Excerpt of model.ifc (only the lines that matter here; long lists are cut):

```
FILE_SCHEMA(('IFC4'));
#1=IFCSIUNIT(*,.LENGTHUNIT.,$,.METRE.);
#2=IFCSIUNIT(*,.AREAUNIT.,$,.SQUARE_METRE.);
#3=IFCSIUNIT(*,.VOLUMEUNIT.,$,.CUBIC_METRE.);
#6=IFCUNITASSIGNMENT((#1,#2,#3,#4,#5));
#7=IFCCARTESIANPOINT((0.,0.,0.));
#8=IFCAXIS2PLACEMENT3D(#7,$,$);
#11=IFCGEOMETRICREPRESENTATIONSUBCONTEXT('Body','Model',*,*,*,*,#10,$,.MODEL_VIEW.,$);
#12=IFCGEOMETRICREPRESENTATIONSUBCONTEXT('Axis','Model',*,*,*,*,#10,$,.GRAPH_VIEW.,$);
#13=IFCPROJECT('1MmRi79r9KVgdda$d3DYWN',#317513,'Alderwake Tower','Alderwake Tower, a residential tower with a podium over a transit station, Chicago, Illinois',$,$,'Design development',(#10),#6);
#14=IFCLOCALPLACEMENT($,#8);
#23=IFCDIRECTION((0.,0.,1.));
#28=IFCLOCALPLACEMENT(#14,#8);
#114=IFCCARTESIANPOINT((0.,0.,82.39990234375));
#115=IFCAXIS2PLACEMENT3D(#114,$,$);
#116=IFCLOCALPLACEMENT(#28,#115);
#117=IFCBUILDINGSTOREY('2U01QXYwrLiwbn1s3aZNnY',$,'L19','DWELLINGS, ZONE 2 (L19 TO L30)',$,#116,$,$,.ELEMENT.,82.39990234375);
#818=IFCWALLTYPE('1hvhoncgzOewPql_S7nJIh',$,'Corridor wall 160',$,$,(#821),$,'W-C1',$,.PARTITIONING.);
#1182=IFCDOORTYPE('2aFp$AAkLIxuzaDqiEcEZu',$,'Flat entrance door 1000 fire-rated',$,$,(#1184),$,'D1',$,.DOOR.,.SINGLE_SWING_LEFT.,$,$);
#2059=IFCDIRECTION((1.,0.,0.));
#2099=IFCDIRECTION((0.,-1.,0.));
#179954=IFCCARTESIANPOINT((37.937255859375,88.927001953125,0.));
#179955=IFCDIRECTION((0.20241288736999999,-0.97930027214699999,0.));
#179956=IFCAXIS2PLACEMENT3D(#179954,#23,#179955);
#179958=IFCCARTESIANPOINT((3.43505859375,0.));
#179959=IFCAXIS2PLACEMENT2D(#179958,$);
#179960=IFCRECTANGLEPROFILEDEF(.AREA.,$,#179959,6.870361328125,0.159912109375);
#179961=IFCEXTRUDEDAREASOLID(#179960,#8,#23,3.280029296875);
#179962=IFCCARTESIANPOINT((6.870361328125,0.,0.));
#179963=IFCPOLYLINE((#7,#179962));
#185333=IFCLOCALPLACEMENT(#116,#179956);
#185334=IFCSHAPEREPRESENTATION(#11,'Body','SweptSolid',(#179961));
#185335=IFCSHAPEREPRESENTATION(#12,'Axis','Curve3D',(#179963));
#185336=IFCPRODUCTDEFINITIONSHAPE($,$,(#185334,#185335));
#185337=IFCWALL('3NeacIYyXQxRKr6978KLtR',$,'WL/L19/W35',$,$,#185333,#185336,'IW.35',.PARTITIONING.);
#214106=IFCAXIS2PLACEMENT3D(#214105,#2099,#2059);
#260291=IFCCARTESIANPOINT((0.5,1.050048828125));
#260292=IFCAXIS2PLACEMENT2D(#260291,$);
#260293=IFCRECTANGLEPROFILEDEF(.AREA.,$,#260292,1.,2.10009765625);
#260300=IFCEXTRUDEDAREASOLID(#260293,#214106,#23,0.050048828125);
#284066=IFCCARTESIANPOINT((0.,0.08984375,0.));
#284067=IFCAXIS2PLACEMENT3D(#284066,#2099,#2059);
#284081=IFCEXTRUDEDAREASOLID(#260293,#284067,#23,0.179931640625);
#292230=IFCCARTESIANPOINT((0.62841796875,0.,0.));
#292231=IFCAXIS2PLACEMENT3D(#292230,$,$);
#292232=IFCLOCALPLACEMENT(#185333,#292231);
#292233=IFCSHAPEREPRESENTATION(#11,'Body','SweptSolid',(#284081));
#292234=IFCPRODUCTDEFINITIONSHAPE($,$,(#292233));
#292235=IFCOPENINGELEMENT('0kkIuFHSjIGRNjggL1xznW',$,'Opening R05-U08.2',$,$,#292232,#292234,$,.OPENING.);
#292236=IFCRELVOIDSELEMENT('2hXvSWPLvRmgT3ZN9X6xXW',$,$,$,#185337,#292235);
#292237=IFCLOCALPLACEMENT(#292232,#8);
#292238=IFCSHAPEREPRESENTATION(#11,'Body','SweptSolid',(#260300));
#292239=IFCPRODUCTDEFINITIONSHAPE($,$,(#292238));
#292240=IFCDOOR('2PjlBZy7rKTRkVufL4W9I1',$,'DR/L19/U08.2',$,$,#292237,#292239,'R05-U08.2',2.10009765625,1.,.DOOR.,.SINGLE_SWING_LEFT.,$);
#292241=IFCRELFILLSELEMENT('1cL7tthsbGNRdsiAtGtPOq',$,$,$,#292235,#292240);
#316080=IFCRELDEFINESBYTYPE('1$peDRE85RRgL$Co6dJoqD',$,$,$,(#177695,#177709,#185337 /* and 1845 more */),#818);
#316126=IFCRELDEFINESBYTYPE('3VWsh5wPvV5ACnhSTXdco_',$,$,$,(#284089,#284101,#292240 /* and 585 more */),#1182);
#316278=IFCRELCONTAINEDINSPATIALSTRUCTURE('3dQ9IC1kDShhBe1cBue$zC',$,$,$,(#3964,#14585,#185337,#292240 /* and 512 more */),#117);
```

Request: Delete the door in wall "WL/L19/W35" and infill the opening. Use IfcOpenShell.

```python
import ifcopenshell
import ifcopenshell.api.feature
import ifcopenshell.api.root
import ifcopenshell.geom
import ifcopenshell.util.shape

model = ifcopenshell.open("model.ifc")
settings = ifcopenshell.geom.settings()


def volume(element):
    """Net volume in cubic metres, openings subtracted."""
    shape = ifcopenshell.geom.create_shape(settings, element)
    return ifcopenshell.util.shape.get_volume(shape.geometry)


door = model.by_guid("2PjlBZy7rKTRkVufL4W9I1")
opening = door.FillsVoids[0].RelatingOpeningElement
wall = opening.VoidsElements[0].RelatingBuildingElement
before = volume(wall)

ifcopenshell.api.root.remove_product(model, product=door)
ifcopenshell.api.feature.remove_feature(model, feature=opening)

after = volume(wall)

print(f"wall volume {before:.3f} -> {after:.3f} m3")

model.write("model_edited.ifc")
```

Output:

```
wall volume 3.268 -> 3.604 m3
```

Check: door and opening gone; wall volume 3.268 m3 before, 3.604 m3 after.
